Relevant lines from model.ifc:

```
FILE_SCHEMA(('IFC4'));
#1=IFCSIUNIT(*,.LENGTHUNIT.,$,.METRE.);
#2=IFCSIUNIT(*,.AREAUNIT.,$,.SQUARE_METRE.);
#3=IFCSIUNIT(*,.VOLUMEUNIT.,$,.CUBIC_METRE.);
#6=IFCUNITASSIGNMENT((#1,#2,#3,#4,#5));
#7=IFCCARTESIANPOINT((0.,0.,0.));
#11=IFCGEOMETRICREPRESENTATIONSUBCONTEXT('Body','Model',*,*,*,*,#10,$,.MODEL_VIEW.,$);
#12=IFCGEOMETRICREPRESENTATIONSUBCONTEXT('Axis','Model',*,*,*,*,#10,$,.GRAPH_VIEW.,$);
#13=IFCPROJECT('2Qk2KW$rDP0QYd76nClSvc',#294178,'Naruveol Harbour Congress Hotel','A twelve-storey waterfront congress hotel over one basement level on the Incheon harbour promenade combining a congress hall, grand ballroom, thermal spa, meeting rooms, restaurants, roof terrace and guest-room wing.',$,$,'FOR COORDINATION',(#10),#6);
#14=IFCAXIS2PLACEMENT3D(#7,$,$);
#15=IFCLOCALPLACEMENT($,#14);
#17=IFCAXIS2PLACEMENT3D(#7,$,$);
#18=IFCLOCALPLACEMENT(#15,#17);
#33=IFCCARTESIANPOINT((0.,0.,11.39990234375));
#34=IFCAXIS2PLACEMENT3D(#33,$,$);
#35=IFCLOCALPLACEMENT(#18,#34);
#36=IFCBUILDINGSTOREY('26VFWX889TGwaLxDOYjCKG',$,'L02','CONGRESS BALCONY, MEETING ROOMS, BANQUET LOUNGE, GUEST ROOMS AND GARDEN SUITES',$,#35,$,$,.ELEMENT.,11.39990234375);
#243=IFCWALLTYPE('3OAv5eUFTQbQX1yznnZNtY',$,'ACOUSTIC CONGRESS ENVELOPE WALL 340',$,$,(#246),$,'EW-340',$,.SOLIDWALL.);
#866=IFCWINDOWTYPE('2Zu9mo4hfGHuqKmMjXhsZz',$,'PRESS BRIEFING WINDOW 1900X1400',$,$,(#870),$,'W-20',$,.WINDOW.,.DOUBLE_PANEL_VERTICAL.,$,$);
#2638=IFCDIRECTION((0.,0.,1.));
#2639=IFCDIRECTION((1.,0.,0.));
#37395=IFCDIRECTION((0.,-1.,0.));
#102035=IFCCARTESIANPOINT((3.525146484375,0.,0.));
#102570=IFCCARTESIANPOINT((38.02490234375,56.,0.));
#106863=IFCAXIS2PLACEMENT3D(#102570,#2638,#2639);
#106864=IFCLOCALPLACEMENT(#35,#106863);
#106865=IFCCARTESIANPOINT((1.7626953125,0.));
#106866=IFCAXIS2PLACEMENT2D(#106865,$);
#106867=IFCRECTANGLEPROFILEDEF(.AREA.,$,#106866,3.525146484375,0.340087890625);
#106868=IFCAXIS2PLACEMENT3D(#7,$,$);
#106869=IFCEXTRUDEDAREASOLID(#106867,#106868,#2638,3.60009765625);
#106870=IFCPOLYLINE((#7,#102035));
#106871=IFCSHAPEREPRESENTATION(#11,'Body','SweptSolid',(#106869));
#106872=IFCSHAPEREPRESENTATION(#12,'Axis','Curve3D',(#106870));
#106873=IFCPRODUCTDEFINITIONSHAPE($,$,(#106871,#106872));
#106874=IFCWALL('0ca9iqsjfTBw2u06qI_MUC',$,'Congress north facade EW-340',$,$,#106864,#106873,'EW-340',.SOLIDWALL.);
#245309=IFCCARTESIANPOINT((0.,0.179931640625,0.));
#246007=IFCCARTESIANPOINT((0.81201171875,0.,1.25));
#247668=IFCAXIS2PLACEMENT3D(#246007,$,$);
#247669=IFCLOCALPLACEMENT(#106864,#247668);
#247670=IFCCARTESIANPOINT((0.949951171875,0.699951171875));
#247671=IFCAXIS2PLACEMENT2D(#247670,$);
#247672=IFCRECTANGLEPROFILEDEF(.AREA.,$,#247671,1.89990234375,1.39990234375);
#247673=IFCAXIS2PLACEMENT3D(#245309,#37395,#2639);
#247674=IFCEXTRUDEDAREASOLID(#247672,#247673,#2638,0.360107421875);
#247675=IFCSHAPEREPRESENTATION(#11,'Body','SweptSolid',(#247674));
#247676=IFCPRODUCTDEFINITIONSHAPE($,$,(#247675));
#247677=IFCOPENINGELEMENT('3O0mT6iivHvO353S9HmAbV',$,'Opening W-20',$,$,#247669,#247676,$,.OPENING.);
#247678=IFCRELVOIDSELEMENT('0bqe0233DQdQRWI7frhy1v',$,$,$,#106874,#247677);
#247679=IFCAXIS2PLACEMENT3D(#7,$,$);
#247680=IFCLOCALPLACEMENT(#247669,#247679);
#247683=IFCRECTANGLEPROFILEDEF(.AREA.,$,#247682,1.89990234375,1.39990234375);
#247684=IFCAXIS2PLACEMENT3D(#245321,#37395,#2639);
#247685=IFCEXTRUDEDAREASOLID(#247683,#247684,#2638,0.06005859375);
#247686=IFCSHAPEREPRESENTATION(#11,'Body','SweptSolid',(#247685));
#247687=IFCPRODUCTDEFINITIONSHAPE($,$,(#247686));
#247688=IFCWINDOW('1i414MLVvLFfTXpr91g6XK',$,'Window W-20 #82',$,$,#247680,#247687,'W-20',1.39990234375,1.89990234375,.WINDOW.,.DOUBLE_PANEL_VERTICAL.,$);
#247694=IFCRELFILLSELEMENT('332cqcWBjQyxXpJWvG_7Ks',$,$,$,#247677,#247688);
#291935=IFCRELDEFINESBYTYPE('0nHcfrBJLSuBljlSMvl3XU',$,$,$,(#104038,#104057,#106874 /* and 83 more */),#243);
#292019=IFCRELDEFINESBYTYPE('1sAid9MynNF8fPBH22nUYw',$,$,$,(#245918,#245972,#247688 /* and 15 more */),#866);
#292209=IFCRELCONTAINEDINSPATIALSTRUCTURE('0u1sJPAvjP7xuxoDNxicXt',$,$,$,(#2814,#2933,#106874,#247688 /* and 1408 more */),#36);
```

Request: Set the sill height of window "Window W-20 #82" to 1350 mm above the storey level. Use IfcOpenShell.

```python
import numpy as np
import ifcopenshell
import ifcopenshell.api.geometry
import ifcopenshell.geom
import ifcopenshell.util.element
import ifcopenshell.util.placement
import ifcopenshell.util.shape
import ifcopenshell.util.unit

model = ifcopenshell.open("model.ifc")
unit_scale = ifcopenshell.util.unit.calculate_unit_scale(model)

window = model.by_guid("1i414MLVvLFfTXpr91g6XK")
opening = window.FillsVoids[0].RelatingOpeningElement
storey = ifcopenshell.util.element.get_container(window, ifc_class="IfcBuildingStorey")
level = ifcopenshell.util.placement.get_local_placement(storey.ObjectPlacement)[2, 3]

# The opening's origin need not be at the sill, so measure its lowest point.
shape = ifcopenshell.geom.create_shape(ifcopenshell.geom.settings(), opening)
bottom = ifcopenshell.util.shape.get_shape_bottom_elevation(shape, shape.geometry) / unit_scale
dz = level + 1.35 / unit_scale - bottom

shift = np.array([0.0, 0.0, dz])
# The window is placed relative to its opening, so it follows when the opening moves.
matrix = ifcopenshell.util.placement.get_local_placement(opening.ObjectPlacement)
matrix[:3, 3] += shift
ifcopenshell.api.geometry.edit_object_placement(
    model, product=opening, matrix=matrix, is_si=False, should_transform_children=True
)

print(f"moved by {dz * unit_scale:+.3f} m")

model.write("model_v2.ifc")
```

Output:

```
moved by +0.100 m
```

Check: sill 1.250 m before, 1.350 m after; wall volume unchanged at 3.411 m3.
